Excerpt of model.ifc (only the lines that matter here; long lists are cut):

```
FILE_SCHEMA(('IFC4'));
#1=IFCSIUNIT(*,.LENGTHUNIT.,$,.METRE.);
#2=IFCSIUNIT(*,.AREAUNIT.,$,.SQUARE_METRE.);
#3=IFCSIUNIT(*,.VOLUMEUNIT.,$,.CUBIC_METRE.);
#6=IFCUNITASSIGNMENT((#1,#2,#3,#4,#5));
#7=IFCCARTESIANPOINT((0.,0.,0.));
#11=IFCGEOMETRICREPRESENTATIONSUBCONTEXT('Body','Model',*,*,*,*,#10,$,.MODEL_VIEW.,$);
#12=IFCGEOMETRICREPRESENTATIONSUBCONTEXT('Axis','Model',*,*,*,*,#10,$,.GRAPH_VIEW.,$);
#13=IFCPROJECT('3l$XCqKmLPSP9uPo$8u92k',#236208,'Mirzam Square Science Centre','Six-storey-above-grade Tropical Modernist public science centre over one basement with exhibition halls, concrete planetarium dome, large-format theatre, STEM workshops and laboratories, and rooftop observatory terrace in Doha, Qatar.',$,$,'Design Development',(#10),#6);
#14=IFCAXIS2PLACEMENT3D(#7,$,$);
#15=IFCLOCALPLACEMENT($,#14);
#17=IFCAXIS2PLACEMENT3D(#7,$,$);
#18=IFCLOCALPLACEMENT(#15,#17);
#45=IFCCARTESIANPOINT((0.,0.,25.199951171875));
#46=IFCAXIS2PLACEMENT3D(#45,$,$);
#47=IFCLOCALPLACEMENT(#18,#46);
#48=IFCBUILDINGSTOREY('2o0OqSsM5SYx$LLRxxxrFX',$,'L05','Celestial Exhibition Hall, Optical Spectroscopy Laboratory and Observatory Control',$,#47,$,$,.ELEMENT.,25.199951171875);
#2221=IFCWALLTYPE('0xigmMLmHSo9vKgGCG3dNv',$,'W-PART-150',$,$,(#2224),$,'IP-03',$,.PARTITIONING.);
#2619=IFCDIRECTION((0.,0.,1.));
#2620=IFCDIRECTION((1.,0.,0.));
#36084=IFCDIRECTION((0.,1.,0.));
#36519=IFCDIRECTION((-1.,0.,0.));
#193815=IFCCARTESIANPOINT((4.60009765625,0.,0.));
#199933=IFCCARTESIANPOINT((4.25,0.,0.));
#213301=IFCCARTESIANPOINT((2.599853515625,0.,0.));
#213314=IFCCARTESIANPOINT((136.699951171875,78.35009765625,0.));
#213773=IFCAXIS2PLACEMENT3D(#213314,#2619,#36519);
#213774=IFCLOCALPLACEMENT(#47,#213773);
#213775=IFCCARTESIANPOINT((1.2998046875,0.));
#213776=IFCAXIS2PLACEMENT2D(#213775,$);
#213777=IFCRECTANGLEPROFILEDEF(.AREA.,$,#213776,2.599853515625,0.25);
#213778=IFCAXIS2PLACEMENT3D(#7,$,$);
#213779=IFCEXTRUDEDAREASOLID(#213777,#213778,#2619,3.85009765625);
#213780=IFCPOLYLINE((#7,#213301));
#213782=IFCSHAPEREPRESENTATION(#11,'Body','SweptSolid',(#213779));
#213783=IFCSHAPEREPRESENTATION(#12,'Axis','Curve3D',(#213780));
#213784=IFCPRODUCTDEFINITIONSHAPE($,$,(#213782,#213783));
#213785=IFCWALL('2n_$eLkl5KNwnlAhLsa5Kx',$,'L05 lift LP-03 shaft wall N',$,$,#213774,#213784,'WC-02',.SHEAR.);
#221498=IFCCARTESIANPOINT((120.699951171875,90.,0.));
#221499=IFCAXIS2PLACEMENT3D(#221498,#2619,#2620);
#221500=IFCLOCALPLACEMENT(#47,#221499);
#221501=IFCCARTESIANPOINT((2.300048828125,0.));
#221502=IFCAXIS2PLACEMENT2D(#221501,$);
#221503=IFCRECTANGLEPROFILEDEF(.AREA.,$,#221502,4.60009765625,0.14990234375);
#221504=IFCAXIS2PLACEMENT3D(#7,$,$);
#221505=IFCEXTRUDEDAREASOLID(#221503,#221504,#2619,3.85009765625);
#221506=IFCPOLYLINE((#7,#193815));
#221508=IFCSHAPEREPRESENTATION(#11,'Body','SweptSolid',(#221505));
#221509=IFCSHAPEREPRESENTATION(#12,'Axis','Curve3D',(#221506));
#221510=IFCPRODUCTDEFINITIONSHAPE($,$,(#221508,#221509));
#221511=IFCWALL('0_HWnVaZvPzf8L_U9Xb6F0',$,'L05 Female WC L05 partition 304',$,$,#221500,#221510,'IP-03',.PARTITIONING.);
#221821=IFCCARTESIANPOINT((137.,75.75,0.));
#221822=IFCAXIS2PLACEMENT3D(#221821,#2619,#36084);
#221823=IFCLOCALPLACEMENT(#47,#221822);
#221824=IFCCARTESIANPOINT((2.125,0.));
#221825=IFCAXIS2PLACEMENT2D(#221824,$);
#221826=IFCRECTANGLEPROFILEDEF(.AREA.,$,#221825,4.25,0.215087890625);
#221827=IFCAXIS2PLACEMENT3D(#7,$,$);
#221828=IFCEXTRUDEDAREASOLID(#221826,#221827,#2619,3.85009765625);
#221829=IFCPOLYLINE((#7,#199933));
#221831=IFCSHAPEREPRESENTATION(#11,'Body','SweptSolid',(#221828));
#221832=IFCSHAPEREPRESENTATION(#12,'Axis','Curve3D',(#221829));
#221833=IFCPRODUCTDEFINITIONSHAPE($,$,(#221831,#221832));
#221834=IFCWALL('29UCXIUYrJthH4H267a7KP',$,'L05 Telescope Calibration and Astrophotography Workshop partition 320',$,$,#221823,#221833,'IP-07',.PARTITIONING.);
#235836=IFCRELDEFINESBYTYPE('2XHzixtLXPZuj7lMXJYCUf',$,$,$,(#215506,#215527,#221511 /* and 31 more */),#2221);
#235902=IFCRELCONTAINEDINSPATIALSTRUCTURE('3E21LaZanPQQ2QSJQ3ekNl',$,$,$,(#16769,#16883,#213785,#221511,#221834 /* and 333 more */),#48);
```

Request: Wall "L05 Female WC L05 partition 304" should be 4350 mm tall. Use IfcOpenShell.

```python
import ifcopenshell
import ifcopenshell.geom
import ifcopenshell.util.representation
import ifcopenshell.util.shape

model = ifcopenshell.open("model.ifc")
settings = ifcopenshell.geom.settings()


def volume(element):
    """Net volume in cubic metres, openings subtracted."""
    shape = ifcopenshell.geom.create_shape(settings, element)
    return ifcopenshell.util.shape.get_volume(shape.geometry)


wall = model.by_guid("0_HWnVaZvPzf8L_U9Xb6F0")
before = volume(wall)

body = ifcopenshell.util.representation.get_representation(wall, "Model", "Body")
solid = body.Items[0]
old_height = solid.Depth
solid.Depth = 4.35
after = volume(wall)

print(f"height {old_height:g} -> {solid.Depth:g}, volume {before:.3f} -> {after:.3f} m3")

model.write("model-out.ifc")
```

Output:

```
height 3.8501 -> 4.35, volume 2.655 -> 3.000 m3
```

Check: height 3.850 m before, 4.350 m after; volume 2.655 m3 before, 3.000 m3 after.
